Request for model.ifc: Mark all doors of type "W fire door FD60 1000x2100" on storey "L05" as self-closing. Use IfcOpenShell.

First a look at what the model holds.

```python
import ifcopenshell
import ifcopenshell.util.element

model = ifcopenshell.open("model.ifc")
print(model.schema)
storey = next(s for s in model.by_type("IfcBuildingStorey") if s.Name == "L05")
doors = [e for e in ifcopenshell.util.element.get_decomposition(storey) if e.is_a("IfcDoor")]
seen = {}
for e in doors:
    element_type = ifcopenshell.util.element.get_type(e)
    key = (element_type.Name if element_type != e and element_type else None, ifcopenshell.util.element.get_pset(e, "Pset_DoorCommon", "SelfClosing"))
    seen[key] = seen.get(key, 0) + 1
for (name, value), count in sorted(seen.items(), key=str):
    print(count, "x", name, "|", value)
```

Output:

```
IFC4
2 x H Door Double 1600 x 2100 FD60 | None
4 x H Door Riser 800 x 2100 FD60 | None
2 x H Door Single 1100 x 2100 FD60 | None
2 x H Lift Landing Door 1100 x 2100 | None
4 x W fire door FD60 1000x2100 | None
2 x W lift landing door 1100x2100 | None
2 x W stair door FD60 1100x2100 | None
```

```python
import ifcopenshell
import ifcopenshell.api.pset
import ifcopenshell.util.element

model = ifcopenshell.open("model.ifc")

storey = next(s for s in model.by_type("IfcBuildingStorey") if s.Name == "L05")
doors = [e for e in ifcopenshell.util.element.get_decomposition(storey) if e.is_a("IfcDoor")]

count = 0
for e in doors:
    element_type = ifcopenshell.util.element.get_type(e)
    if element_type in (None, e) or element_type.Name != "W fire door FD60 1000x2100":
        continue
    # add_pset returns the element's existing set when there is one.
    pset = ifcopenshell.api.pset.add_pset(model, product=e, name="Pset_DoorCommon")
    ifcopenshell.api.pset.edit_pset(model, pset=pset, properties={"SelfClosing": True})
    count += 1

print(count, "doors updated")

model.write("model_updated.ifc")
```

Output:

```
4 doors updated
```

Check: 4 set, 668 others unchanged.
